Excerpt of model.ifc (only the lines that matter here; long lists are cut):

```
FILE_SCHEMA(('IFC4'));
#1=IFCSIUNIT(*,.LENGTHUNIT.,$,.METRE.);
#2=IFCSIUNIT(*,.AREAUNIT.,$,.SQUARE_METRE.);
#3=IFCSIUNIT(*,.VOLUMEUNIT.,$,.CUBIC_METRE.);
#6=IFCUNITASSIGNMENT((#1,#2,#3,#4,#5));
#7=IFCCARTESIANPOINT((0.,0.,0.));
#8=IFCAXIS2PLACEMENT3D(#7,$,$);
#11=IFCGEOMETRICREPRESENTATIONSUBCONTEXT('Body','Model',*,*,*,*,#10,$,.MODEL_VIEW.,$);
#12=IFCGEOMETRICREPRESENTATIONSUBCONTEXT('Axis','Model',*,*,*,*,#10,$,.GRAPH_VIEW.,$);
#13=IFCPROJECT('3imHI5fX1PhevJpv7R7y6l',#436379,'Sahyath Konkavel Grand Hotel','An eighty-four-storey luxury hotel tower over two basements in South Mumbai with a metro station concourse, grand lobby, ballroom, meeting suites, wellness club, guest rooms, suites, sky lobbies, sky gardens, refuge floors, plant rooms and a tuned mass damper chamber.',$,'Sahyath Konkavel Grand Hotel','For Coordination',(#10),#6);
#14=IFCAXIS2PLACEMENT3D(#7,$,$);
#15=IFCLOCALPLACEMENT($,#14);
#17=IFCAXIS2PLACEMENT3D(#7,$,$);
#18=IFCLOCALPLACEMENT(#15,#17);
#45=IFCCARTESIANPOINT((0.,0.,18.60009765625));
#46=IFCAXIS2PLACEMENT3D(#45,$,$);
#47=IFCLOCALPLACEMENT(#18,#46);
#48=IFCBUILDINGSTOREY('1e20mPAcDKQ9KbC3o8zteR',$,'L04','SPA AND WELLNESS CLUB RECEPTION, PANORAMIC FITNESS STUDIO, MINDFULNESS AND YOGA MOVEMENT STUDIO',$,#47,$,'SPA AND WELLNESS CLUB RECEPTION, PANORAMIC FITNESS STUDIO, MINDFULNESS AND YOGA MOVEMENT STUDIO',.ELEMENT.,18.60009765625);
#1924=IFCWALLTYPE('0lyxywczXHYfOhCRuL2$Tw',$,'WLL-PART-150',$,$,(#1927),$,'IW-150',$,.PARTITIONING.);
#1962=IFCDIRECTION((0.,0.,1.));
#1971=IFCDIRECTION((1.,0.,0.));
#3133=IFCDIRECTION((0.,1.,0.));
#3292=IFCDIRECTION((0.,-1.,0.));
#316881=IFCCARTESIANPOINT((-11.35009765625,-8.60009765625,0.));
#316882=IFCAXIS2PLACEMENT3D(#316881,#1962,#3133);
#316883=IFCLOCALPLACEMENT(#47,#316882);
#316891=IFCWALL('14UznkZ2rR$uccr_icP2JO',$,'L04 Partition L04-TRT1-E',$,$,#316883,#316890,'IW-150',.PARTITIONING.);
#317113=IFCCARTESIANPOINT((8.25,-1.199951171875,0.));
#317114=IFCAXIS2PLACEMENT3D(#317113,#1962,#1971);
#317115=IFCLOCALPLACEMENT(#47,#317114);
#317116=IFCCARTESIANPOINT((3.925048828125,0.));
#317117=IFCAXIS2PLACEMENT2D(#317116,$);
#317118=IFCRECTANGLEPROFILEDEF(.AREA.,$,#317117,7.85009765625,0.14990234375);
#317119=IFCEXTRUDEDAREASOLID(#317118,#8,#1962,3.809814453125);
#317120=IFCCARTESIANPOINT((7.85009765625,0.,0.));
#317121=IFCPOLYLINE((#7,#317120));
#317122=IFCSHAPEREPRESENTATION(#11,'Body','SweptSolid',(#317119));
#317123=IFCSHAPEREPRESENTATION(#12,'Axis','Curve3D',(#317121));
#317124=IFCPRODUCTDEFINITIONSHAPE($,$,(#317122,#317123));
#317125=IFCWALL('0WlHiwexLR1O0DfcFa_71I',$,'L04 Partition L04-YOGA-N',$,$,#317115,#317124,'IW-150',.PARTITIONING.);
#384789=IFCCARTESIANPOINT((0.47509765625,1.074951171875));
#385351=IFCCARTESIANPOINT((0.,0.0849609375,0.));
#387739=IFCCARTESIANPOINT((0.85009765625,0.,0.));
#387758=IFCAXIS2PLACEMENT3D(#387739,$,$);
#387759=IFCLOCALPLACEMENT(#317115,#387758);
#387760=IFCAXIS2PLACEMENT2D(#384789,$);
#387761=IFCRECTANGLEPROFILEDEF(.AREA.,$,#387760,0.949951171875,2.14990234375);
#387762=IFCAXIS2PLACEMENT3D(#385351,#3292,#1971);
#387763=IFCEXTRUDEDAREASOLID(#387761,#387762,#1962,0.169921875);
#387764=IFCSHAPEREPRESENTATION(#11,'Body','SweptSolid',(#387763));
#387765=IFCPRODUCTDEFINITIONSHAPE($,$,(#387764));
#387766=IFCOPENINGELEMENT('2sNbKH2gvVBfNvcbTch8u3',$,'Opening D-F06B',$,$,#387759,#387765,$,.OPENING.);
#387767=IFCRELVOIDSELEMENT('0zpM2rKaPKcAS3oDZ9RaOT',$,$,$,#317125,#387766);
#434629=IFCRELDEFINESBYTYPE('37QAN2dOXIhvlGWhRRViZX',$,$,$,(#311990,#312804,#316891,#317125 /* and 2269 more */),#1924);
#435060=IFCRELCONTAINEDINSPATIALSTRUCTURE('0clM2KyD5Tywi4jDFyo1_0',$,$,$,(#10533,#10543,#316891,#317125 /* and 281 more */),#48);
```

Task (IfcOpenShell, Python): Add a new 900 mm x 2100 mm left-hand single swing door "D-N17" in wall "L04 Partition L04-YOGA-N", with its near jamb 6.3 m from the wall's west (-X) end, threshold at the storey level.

```python
import numpy as np
import ifcopenshell
import ifcopenshell.api.feature
import ifcopenshell.api.geometry
import ifcopenshell.api.root
import ifcopenshell.api.spatial
import ifcopenshell.geom
import ifcopenshell.util.element
import ifcopenshell.util.placement
import ifcopenshell.util.representation
import ifcopenshell.util.shape
import ifcopenshell.util.unit

model = ifcopenshell.open("model.ifc")
unit_scale = ifcopenshell.util.unit.calculate_unit_scale(model)
settings = ifcopenshell.geom.settings()


def volume(element):
    """Net volume in cubic metres, openings subtracted."""
    shape = ifcopenshell.geom.create_shape(settings, element)
    return ifcopenshell.util.shape.get_volume(shape.geometry)


wall = model.by_guid("0WlHiwexLR1O0DfcFa_71I")
storey = ifcopenshell.util.element.get_container(wall, ifc_class="IfcBuildingStorey")
context = ifcopenshell.util.representation.get_context(model, "Model", "Body", "MODEL_VIEW")
before = volume(wall)

width, height, from_end, sill = 0.9, 2.1, 6.3, 0.0  # metres

# The wall runs along its own X axis, and the end named is its -X end.
wall_shape = ifcopenshell.geom.create_shape(settings, wall)
x, y, z = ifcopenshell.util.shape.get_vertices(wall_shape.geometry).T
start = x.min() + from_end
face, thickness = float(y.min()), float(y.max() - y.min())
wall_matrix = ifcopenshell.util.placement.get_local_placement(wall.ObjectPlacement)
level = ifcopenshell.util.placement.get_local_placement(storey.ObjectPlacement)[2, 3]


def in_wall(x, y):
    """Placement at x, y metres in the wall's axes, at sill height."""
    matrix = wall_matrix.copy()
    matrix[:, 3] = wall_matrix @ np.array([x / unit_scale, y / unit_scale, 0.0, 1.0])
    matrix[2, 3] = level + sill / unit_scale
    return matrix


# Opening: a box that overshoots both wall faces by 50 mm.
opening = ifcopenshell.api.root.create_entity(model, ifc_class="IfcOpeningElement", predefined_type="OPENING")
box = ifcopenshell.api.geometry.add_wall_representation(
    model, context=context, length=width, height=height, thickness=thickness + 0.1
)
ifcopenshell.api.geometry.assign_representation(model, product=opening, representation=box)
ifcopenshell.api.geometry.edit_object_placement(model, product=opening, matrix=in_wall(start, face - 0.05), is_si=False)
ifcopenshell.api.feature.add_feature(model, feature=opening, element=wall)

door = ifcopenshell.api.root.create_entity(model, ifc_class="IfcDoor", name="D-N17", predefined_type="DOOR")
door.OverallWidth, door.OverallHeight = width / unit_scale, height / unit_scale
door.OperationType = "SINGLE_SWING_LEFT"
body = ifcopenshell.api.geometry.add_door_representation(
    model,
    context=context,
    overall_width=door.OverallWidth,
    overall_height=door.OverallHeight,
    operation_type="SINGLE_SWING_LEFT",
    lining_properties={"LiningDepth": thickness / unit_scale, "ThresholdDepth": thickness / unit_scale},
)
ifcopenshell.api.geometry.assign_representation(model, product=door, representation=body)
ifcopenshell.api.spatial.assign_container(model, products=[door], relating_structure=storey)
ifcopenshell.api.feature.add_filling(model, opening=opening, element=door)

# The lining spans the wall, so the door starts at the wall face.
ifcopenshell.api.geometry.edit_object_placement(model, product=door, matrix=in_wall(start, face), is_si=False)

after = volume(wall)

print(f"wall volume {before:.3f} -> {after:.3f} m3")

model.write("model_updated.ifc")
```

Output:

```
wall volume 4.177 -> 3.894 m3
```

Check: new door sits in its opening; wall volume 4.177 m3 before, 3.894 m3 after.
